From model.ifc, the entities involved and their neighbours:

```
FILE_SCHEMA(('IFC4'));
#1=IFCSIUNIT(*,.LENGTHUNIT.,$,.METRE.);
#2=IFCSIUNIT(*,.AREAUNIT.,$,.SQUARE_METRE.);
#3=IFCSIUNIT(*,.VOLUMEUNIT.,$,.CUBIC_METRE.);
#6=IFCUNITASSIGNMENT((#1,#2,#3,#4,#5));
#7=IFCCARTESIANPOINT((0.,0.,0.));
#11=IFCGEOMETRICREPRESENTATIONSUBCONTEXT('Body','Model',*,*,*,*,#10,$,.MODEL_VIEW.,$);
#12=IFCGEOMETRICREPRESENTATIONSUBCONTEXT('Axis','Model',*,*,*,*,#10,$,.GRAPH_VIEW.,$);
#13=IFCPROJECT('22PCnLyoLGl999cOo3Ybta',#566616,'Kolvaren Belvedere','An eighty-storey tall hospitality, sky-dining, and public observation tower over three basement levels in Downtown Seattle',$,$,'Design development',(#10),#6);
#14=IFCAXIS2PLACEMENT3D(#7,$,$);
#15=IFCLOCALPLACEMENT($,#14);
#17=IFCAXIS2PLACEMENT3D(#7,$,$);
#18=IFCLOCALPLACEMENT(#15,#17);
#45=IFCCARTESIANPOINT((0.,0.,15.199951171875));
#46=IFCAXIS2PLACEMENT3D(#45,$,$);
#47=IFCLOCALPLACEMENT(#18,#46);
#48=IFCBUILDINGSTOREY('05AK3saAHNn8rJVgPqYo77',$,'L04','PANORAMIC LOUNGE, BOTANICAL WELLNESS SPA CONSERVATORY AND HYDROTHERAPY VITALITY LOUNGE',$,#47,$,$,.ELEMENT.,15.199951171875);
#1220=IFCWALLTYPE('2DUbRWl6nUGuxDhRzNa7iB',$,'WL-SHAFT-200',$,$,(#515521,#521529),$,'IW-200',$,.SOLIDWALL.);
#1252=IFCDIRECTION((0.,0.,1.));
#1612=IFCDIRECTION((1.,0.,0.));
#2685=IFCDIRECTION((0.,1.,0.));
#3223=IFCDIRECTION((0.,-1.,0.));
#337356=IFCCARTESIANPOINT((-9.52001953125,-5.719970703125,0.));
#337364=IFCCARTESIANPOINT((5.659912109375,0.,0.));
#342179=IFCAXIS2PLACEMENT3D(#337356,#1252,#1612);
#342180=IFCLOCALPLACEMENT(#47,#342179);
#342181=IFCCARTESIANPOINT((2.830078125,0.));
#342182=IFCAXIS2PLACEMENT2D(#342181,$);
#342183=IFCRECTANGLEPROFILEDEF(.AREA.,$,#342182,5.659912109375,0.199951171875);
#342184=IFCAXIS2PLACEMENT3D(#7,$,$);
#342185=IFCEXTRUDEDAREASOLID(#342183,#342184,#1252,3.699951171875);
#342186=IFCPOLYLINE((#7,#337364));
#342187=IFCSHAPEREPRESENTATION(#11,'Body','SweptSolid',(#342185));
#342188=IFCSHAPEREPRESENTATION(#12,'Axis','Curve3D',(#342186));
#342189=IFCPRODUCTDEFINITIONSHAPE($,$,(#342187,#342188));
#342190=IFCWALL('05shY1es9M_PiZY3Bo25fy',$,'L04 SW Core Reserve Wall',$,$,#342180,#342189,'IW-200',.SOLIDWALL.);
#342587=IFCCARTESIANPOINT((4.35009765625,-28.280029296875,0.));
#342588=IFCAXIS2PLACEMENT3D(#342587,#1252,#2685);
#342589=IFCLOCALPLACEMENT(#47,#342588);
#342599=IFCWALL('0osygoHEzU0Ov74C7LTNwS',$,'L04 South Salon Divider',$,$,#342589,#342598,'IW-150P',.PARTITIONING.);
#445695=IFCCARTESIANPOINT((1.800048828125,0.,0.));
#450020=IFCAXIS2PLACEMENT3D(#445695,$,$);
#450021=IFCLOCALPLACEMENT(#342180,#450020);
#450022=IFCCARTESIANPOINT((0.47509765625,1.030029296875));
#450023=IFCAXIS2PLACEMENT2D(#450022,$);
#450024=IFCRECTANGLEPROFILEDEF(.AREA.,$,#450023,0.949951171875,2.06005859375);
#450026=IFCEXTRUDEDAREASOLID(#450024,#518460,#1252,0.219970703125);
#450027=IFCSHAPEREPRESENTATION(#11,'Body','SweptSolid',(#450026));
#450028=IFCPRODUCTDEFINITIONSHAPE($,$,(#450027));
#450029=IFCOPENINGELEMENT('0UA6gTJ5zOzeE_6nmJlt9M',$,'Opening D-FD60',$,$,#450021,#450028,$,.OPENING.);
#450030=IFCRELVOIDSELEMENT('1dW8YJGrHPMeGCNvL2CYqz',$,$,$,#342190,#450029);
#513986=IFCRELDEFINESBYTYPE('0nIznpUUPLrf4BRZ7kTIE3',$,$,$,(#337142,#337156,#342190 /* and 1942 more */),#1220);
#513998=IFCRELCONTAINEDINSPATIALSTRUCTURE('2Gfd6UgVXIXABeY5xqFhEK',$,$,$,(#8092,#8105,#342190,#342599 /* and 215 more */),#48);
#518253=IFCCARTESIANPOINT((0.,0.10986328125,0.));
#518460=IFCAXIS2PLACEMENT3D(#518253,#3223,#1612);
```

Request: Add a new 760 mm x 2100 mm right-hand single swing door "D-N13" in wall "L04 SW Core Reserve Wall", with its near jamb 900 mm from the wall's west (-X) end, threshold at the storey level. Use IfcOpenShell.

```python
import numpy as np
import ifcopenshell
import ifcopenshell.api.feature
import ifcopenshell.api.geometry
import ifcopenshell.api.root
import ifcopenshell.api.spatial
import ifcopenshell.geom
import ifcopenshell.util.element
import ifcopenshell.util.placement
import ifcopenshell.util.representation
import ifcopenshell.util.shape
import ifcopenshell.util.unit

model = ifcopenshell.open("model.ifc")
unit_scale = ifcopenshell.util.unit.calculate_unit_scale(model)
settings = ifcopenshell.geom.settings()


def volume(element):
    """Net volume in cubic metres, openings subtracted."""
    shape = ifcopenshell.geom.create_shape(settings, element)
    return ifcopenshell.util.shape.get_volume(shape.geometry)


wall = model.by_guid("05shY1es9M_PiZY3Bo25fy")
storey = ifcopenshell.util.element.get_container(wall, ifc_class="IfcBuildingStorey")
context = ifcopenshell.util.representation.get_context(model, "Model", "Body", "MODEL_VIEW")
before = volume(wall)

width, height, from_end, sill = 0.76, 2.1, 0.9, 0.0  # metres

# The wall runs along its own X axis, and the end named is its -X end.
wall_shape = ifcopenshell.geom.create_shape(settings, wall)
x, y, z = ifcopenshell.util.shape.get_vertices(wall_shape.geometry).T
start = x.min() + from_end
face, thickness = float(y.min()), float(y.max() - y.min())
wall_matrix = ifcopenshell.util.placement.get_local_placement(wall.ObjectPlacement)
level = ifcopenshell.util.placement.get_local_placement(storey.ObjectPlacement)[2, 3]


def in_wall(x, y):
    """Placement at x, y metres in the wall's axes, at sill height."""
    matrix = wall_matrix.copy()
    matrix[:, 3] = wall_matrix @ np.array([x / unit_scale, y / unit_scale, 0.0, 1.0])
    matrix[2, 3] = level + sill / unit_scale
    return matrix


# Opening: a box that overshoots both wall faces by 50 mm.
opening = ifcopenshell.api.root.create_entity(model, ifc_class="IfcOpeningElement", predefined_type="OPENING")
box = ifcopenshell.api.geometry.add_wall_representation(
    model, context=context, length=width, height=height, thickness=thickness + 0.1
)
ifcopenshell.api.geometry.assign_representation(model, product=opening, representation=box)
ifcopenshell.api.geometry.edit_object_placement(model, product=opening, matrix=in_wall(start, face - 0.05), is_si=False)
ifcopenshell.api.feature.add_feature(model, feature=opening, element=wall)

door = ifcopenshell.api.root.create_entity(model, ifc_class="IfcDoor", name="D-N13", predefined_type="DOOR")
door.OverallWidth, door.OverallHeight = width / unit_scale, height / unit_scale
door.OperationType = "SINGLE_SWING_RIGHT"
body = ifcopenshell.api.geometry.add_door_representation(
    model,
    context=context,
    overall_width=door.OverallWidth,
    overall_height=door.OverallHeight,
    operation_type="SINGLE_SWING_RIGHT",
    lining_properties={"LiningDepth": thickness / unit_scale, "ThresholdDepth": thickness / unit_scale},
)
ifcopenshell.api.geometry.assign_representation(model, product=door, representation=body)
ifcopenshell.api.spatial.assign_container(model, products=[door], relating_structure=storey)
ifcopenshell.api.feature.add_filling(model, opening=opening, element=door)

# The lining spans the wall, so the door starts at the wall face.
ifcopenshell.api.geometry.edit_object_placement(model, product=door, matrix=in_wall(start, face), is_si=False)

after = volume(wall)

print(f"wall volume {before:.3f} -> {after:.3f} m3")

model.write("model-out.ifc")
```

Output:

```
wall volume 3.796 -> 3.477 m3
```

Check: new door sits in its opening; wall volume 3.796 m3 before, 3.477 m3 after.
